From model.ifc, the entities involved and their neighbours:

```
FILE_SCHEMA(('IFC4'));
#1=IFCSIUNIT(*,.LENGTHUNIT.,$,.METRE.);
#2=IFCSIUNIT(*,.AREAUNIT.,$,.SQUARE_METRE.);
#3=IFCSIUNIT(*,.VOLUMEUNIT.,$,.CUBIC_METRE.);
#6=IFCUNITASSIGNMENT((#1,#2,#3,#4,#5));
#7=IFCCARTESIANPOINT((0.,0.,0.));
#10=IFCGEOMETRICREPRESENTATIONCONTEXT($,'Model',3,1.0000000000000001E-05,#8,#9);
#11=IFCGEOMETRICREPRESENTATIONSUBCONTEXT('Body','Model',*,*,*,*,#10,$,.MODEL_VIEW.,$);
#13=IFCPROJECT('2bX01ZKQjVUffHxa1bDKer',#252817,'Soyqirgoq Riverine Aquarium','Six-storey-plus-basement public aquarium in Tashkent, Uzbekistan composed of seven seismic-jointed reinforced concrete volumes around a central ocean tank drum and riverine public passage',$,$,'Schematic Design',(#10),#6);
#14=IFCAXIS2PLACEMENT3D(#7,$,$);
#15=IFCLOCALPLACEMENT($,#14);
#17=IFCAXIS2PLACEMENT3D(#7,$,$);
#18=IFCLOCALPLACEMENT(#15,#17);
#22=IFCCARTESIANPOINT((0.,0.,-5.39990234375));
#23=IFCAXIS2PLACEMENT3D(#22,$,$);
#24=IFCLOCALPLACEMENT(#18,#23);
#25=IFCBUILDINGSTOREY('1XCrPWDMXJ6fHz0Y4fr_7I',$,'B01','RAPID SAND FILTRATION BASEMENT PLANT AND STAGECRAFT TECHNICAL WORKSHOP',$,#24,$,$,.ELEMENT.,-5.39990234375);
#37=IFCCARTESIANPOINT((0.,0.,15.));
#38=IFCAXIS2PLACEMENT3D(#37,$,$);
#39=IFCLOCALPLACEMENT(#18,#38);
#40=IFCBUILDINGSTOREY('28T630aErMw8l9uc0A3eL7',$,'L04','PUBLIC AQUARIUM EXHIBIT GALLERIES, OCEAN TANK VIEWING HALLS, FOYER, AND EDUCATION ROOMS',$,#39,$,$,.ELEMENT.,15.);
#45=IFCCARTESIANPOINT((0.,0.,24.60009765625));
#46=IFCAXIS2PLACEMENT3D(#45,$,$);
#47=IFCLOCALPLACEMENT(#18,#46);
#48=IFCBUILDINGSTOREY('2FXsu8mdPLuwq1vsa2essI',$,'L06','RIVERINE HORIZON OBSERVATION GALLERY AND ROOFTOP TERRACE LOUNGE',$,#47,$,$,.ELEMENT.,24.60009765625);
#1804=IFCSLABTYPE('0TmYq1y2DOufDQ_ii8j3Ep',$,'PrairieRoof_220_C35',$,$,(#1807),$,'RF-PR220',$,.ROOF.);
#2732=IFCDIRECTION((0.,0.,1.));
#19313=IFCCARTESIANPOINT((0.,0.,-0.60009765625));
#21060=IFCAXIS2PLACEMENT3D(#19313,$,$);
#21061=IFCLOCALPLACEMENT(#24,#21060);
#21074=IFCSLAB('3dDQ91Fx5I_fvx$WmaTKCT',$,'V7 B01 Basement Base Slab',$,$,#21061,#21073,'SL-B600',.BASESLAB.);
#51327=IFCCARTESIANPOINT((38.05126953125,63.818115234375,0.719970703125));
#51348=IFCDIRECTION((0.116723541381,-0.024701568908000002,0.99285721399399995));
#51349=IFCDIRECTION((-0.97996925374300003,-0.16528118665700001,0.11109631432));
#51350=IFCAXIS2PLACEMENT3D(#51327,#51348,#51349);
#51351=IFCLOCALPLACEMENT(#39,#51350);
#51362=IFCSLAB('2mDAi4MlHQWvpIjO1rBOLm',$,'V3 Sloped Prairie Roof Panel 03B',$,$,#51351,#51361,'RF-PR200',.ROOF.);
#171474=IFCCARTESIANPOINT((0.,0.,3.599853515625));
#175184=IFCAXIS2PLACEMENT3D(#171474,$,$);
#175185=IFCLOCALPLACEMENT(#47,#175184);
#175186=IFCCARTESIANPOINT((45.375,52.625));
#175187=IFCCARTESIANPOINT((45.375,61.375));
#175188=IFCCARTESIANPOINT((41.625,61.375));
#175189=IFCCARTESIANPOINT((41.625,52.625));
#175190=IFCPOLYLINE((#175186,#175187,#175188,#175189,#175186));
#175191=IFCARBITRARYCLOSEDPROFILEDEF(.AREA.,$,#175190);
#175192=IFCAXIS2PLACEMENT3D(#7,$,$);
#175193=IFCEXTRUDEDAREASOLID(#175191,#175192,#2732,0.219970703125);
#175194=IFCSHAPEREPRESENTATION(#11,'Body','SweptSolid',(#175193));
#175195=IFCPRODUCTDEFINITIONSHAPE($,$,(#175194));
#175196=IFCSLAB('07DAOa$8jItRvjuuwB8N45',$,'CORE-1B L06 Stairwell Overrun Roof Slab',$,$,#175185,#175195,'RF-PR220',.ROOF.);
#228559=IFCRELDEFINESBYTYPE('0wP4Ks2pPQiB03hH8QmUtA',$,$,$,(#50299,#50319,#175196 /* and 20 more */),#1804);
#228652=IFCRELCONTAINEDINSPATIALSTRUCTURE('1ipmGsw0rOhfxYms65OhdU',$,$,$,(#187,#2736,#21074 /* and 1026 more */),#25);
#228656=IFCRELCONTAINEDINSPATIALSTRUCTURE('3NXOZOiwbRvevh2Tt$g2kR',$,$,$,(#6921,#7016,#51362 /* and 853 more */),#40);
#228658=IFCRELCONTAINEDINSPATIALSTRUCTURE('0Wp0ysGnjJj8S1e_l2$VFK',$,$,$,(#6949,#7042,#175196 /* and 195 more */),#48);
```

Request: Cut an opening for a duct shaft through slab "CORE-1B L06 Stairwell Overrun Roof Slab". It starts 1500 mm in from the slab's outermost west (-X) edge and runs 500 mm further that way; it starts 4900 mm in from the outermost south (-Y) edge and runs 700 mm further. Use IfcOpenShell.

```python
import numpy as np
import ifcopenshell
import ifcopenshell.api.feature
import ifcopenshell.api.geometry
import ifcopenshell.api.root
import ifcopenshell.geom
import ifcopenshell.util.placement
import ifcopenshell.util.representation
import ifcopenshell.util.shape
import ifcopenshell.util.unit

model = ifcopenshell.open("model.ifc")
unit_scale = ifcopenshell.util.unit.calculate_unit_scale(model)
settings = ifcopenshell.geom.settings()


def volume(element):
    """Net volume in cubic metres, openings subtracted."""
    shape = ifcopenshell.geom.create_shape(settings, element)
    return ifcopenshell.util.shape.get_volume(shape.geometry)


slab = model.by_guid("07DAOa$8jItRvjuuwB8N45")
before = volume(slab)

# Extent in the slab's own axes, in metres. The edges named are its -X and -Y sides.
slab_shape = ifcopenshell.geom.create_shape(settings, slab)
vertices = ifcopenshell.util.shape.get_vertices(slab_shape.geometry)
x_min, y_min, bottom = vertices.min(axis=0)
top = vertices[:, 2].max()

opening = ifcopenshell.api.root.create_entity(model, ifc_class="IfcOpeningElement", name="Duct shaft opening", predefined_type="OPENING")
context = ifcopenshell.util.representation.get_context(model, "Model", "Body", "MODEL_VIEW")
width, depth = 0.5, 0.7
outline = [(0.0, 0.0), (width, 0.0), (width, depth), (0.0, depth), (0.0, 0.0)]
# Overshoot both faces by 50 mm so the cut is clean.
shape = ifcopenshell.api.geometry.add_slab_representation(
    model, context=context, depth=top - bottom + 0.1, polyline=outline
)
ifcopenshell.api.geometry.assign_representation(model, product=opening, representation=shape)

matrix = ifcopenshell.util.placement.get_local_placement(slab.ObjectPlacement)
matrix[:, 3] = matrix @ np.append(np.array([x_min + 1.5, y_min + 4.9, bottom - 0.05]) / unit_scale, 1.0)
ifcopenshell.api.geometry.edit_object_placement(model, product=opening, matrix=matrix, is_si=False)
ifcopenshell.api.feature.add_feature(model, feature=opening, element=slab)

after = volume(slab)

print(f"slab volume {before:.3f} -> {after:.3f} m3")

model.write("model_rev.ifc")
```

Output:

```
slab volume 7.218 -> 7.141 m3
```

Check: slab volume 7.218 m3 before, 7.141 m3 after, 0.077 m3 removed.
